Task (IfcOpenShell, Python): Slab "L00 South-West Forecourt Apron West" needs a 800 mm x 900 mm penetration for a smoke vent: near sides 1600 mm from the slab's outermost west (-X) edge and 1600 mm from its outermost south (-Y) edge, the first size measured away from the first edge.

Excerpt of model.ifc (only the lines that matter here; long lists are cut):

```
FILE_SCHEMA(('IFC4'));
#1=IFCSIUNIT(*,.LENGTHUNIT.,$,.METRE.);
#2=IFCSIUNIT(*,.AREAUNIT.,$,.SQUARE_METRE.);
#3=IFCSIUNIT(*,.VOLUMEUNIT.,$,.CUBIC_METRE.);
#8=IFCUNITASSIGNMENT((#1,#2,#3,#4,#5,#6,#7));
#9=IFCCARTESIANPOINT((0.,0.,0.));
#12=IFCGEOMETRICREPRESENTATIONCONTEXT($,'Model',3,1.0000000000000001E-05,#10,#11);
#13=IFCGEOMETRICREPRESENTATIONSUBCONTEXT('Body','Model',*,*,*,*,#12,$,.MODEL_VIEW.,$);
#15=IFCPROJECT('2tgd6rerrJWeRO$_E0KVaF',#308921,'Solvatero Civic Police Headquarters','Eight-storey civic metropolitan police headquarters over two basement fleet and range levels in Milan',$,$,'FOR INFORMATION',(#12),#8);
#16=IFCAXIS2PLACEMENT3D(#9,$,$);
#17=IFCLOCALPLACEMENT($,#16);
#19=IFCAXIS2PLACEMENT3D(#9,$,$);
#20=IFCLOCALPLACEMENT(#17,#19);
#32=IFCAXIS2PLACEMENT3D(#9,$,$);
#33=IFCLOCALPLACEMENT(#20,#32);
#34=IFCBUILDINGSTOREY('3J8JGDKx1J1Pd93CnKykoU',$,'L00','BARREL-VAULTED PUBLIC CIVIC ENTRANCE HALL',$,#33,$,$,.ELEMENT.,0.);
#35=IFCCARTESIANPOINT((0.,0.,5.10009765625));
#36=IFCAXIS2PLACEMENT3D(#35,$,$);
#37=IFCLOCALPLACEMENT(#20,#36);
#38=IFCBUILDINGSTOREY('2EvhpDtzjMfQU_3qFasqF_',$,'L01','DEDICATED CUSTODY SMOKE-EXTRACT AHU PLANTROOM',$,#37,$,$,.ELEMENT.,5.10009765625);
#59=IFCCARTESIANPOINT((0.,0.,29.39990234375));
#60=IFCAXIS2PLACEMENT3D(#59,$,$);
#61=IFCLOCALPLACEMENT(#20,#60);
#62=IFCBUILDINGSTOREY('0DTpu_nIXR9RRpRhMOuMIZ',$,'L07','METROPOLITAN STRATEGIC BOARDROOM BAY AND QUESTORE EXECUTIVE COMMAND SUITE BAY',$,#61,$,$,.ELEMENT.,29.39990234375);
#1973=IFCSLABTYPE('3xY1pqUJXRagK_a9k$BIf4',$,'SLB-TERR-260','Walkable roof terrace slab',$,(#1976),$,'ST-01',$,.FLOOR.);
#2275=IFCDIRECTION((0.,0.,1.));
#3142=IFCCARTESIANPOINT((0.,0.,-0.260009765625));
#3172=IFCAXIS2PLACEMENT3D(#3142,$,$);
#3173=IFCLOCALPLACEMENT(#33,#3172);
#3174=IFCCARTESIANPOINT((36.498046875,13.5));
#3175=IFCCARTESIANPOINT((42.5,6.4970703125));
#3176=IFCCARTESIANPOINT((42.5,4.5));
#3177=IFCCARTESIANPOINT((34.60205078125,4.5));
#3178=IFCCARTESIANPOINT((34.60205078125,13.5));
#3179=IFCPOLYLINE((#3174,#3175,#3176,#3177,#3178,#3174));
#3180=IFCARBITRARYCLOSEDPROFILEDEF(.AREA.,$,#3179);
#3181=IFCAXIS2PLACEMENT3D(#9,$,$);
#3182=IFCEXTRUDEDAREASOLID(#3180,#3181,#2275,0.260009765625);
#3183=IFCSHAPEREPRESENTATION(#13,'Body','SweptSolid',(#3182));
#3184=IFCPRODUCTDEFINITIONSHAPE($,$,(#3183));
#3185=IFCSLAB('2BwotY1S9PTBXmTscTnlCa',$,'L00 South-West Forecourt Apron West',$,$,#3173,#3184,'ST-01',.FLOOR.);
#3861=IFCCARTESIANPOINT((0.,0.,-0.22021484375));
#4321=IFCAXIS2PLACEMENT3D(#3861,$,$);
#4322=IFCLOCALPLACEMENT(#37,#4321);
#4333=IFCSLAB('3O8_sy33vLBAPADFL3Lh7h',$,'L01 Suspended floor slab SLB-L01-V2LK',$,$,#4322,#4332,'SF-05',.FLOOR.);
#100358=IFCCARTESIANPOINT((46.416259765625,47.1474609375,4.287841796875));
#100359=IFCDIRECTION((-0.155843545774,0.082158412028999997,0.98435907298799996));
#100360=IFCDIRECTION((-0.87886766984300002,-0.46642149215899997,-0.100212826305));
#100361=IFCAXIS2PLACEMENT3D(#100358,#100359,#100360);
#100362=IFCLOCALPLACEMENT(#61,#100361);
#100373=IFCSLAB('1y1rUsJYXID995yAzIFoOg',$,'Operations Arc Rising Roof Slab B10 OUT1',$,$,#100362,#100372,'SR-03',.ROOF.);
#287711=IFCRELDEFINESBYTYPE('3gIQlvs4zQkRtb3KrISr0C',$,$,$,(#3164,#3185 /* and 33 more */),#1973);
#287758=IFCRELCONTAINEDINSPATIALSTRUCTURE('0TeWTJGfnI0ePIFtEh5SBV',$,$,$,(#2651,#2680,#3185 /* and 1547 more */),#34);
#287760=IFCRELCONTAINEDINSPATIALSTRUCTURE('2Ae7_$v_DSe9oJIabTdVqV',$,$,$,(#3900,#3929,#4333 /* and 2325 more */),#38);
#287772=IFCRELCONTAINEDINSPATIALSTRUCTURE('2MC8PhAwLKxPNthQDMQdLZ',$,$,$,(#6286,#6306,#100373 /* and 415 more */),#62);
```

```python
import numpy as np
import ifcopenshell
import ifcopenshell.api.feature
import ifcopenshell.api.geometry
import ifcopenshell.api.root
import ifcopenshell.geom
import ifcopenshell.util.placement
import ifcopenshell.util.representation
import ifcopenshell.util.shape
import ifcopenshell.util.unit

model = ifcopenshell.open("model.ifc")
unit_scale = ifcopenshell.util.unit.calculate_unit_scale(model)
settings = ifcopenshell.geom.settings()


def volume(element):
    """Net volume in cubic metres, openings subtracted."""
    shape = ifcopenshell.geom.create_shape(settings, element)
    return ifcopenshell.util.shape.get_volume(shape.geometry)


slab = model.by_guid("2BwotY1S9PTBXmTscTnlCa")
before = volume(slab)

# Extent in the slab's own axes, in metres. The edges named are its -X and -Y sides.
slab_shape = ifcopenshell.geom.create_shape(settings, slab)
vertices = ifcopenshell.util.shape.get_vertices(slab_shape.geometry)
x_min, y_min, bottom = vertices.min(axis=0)
top = vertices[:, 2].max()

opening = ifcopenshell.api.root.create_entity(model, ifc_class="IfcOpeningElement", name="Smoke vent opening", predefined_type="OPENING")
context = ifcopenshell.util.representation.get_context(model, "Model", "Body", "MODEL_VIEW")
width, depth = 0.8, 0.9
outline = [(0.0, 0.0), (width, 0.0), (width, depth), (0.0, depth), (0.0, 0.0)]
# Overshoot both faces by 50 mm so the cut is clean.
shape = ifcopenshell.api.geometry.add_slab_representation(
    model, context=context, depth=top - bottom + 0.1, polyline=outline
)
ifcopenshell.api.geometry.assign_representation(model, product=opening, representation=shape)

matrix = ifcopenshell.util.placement.get_local_placement(slab.ObjectPlacement)
matrix[:, 3] = matrix @ np.append(np.array([x_min + 1.6, y_min + 1.6, bottom - 0.05]) / unit_scale, 1.0)
ifcopenshell.api.geometry.edit_object_placement(model, product=opening, matrix=matrix, is_si=False)
ifcopenshell.api.feature.add_feature(model, feature=opening, element=slab)

after = volume(slab)

print(f"slab volume {before:.3f} -> {after:.3f} m3")

model.write("model-out.ifc")
```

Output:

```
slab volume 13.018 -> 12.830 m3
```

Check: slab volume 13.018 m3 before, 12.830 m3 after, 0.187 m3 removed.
